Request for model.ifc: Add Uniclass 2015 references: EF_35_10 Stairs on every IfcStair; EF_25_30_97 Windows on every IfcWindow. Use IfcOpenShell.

First a look at what the model holds.

```python
import ifcopenshell

model = ifcopenshell.open("model.ifc")
print(model.schema)
print("classifications:", [c.Name for c in model.by_type("IfcClassification")])
for ifc_class in ("IfcDoor", "IfcRoof", "IfcStair", "IfcWall", "IfcWindow"):
    print(ifc_class, len(model.by_type(ifc_class)))
```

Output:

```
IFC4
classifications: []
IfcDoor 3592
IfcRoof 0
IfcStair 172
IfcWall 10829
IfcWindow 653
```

```python
import ifcopenshell
import ifcopenshell.api.classification

model = ifcopenshell.open("model.ifc")

system = ifcopenshell.api.classification.add_classification(model, classification="Uniclass 2015")

codes = {
    "IfcStair": ("EF_35_10", "Stairs"),
    "IfcWindow": ("EF_25_30_97", "Windows"),
}
for ifc_class, (code, name) in codes.items():
    products = model.by_type(ifc_class)
    ifcopenshell.api.classification.add_reference(
        model, products=products, classification=system, identification=code, name=name
    )
    print(code, len(products))

model.write("model_rev.ifc")
```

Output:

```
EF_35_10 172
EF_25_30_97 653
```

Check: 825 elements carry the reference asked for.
